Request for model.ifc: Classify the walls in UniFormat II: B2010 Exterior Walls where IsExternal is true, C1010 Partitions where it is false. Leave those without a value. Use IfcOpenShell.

First a look at what the model holds.

```python
import ifcopenshell
import ifcopenshell.util.element

model = ifcopenshell.open("model.ifc")
print(model.schema)
print("classifications:", [c.Name for c in model.by_type("IfcClassification")])
values = [ifcopenshell.util.element.get_pset(e, "Pset_WallCommon", "IsExternal") for e in model.by_type("IfcWall")]
for value in (True, False, None):
    print("IsExternal", value, values.count(value))
```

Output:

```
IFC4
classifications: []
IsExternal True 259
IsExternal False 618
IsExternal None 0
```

```python
import ifcopenshell
import ifcopenshell.api.classification
import ifcopenshell.util.element

model = ifcopenshell.open("model.ifc")

system = ifcopenshell.api.classification.add_classification(model, classification="UniFormat II")

walls = model.by_type("IfcWall")
external = {e: ifcopenshell.util.element.get_pset(e, "Pset_WallCommon", "IsExternal") for e in walls}
for flag, code, name in ((True, "B2010", "Exterior Walls"), (False, "C1010", "Partitions")):
    products = [e for e in walls if external[e] is flag]
    ifcopenshell.api.classification.add_reference(
        model, products=products, classification=system, identification=code, name=name
    )
    print(code, len(products))

model.write("model-out.ifc")
```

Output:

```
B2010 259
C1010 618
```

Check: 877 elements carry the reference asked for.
